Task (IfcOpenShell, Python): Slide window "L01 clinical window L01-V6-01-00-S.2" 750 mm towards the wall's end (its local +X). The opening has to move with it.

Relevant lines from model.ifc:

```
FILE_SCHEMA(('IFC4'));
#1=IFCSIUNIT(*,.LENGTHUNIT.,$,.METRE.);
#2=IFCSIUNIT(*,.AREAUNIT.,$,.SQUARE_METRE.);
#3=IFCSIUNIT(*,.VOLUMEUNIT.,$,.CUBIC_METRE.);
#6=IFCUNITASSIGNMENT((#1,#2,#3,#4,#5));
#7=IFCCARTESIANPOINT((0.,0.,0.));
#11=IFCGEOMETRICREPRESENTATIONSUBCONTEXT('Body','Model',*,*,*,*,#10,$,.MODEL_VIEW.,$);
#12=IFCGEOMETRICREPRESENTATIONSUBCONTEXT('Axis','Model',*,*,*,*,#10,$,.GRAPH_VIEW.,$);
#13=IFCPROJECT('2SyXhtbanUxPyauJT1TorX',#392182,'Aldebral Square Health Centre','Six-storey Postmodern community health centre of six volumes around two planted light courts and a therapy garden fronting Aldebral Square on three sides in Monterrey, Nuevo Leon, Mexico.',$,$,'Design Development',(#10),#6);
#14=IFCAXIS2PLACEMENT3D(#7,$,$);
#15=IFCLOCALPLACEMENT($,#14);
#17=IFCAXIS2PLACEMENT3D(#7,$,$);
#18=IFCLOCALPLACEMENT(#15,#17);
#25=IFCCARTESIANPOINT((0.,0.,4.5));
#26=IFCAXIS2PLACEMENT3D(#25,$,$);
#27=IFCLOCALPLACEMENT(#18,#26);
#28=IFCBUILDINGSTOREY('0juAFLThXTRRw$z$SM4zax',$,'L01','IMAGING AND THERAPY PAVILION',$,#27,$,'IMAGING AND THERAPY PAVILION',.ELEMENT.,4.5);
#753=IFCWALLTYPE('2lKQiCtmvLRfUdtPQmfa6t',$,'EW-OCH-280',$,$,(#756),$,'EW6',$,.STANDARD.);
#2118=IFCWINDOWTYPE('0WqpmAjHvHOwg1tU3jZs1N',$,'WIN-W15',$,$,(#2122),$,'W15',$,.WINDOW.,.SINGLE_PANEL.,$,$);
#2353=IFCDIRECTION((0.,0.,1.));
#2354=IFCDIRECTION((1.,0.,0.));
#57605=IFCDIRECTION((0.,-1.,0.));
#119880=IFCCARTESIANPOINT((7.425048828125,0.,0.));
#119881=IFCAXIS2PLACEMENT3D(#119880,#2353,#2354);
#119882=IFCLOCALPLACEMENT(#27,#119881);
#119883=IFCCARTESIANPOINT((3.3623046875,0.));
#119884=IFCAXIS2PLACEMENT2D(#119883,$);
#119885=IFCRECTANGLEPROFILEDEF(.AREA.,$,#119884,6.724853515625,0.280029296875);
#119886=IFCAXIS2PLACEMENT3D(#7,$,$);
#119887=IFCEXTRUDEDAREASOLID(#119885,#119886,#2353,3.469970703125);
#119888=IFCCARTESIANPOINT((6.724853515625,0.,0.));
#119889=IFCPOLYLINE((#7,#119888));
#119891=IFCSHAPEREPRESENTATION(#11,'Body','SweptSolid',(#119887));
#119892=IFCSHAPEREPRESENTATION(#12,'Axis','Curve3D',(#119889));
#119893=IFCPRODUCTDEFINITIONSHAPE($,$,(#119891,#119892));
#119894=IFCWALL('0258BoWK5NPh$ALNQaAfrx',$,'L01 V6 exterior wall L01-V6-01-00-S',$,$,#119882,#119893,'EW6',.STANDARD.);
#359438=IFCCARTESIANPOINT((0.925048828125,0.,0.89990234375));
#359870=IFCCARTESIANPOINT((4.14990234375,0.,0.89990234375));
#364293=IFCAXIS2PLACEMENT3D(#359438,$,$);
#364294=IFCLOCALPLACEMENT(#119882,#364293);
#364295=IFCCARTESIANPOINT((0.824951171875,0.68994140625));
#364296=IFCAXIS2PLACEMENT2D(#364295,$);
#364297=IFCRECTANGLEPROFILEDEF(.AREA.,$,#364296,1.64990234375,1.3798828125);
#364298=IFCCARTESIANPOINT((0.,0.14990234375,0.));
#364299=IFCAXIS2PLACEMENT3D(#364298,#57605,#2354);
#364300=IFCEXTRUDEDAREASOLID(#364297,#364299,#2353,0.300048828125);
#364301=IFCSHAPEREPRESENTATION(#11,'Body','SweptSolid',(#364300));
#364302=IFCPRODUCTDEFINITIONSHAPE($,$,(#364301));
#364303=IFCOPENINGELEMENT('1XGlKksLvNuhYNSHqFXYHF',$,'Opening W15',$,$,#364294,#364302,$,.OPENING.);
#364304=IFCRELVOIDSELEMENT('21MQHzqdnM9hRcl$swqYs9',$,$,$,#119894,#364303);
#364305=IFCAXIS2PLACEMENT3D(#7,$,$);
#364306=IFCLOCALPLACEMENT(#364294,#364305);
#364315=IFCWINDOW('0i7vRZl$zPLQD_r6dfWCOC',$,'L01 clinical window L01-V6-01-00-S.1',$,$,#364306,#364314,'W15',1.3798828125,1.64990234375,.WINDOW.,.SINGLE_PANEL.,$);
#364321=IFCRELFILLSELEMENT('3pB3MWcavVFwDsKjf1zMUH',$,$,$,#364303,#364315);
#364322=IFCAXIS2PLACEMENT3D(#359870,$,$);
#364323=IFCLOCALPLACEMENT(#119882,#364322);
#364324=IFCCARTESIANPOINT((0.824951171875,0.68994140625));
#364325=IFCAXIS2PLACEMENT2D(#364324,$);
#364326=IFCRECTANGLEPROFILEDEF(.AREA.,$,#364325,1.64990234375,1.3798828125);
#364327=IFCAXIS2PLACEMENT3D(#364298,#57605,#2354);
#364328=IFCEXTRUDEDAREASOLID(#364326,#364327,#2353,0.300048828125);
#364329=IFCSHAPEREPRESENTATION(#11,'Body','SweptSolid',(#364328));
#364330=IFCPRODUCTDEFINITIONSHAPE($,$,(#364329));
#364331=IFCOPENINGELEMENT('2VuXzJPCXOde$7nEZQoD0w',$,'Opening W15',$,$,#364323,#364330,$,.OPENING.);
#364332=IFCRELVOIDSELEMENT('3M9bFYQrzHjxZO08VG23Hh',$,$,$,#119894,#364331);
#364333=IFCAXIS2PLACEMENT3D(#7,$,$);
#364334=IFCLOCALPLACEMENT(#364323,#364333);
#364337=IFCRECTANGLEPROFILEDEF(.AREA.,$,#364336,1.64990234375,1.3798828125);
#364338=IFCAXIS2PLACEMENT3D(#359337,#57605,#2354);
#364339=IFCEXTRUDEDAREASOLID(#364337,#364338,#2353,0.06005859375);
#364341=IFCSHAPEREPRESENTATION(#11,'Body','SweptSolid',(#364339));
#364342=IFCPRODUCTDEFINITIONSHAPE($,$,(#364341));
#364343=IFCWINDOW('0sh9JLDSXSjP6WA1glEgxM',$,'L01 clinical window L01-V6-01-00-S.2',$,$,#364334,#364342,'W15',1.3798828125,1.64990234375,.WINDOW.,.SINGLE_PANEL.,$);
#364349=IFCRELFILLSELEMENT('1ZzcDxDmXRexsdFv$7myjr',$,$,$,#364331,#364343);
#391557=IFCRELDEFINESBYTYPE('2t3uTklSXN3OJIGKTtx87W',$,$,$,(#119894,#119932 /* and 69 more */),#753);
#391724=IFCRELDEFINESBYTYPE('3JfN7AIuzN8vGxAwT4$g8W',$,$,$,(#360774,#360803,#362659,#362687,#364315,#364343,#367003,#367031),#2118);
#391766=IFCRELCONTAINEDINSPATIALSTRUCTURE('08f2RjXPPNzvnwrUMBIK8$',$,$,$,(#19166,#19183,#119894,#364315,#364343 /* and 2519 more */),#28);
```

```python
import ifcopenshell
import ifcopenshell.api.geometry
import ifcopenshell.util.placement
import ifcopenshell.util.unit

model = ifcopenshell.open("model.ifc")
unit_scale = ifcopenshell.util.unit.calculate_unit_scale(model)

window = model.by_guid("0sh9JLDSXSjP6WA1glEgxM")
opening = window.FillsVoids[0].RelatingOpeningElement
wall = opening.VoidsElements[0].RelatingBuildingElement

wall_matrix = ifcopenshell.util.placement.get_local_placement(wall.ObjectPlacement)
shift = wall_matrix[:3, 0] * 0.75 / unit_scale
before = ifcopenshell.util.placement.get_local_placement(window.ObjectPlacement)[:3, 3].copy()

# The window is placed relative to its opening, so it follows when the opening moves.
matrix = ifcopenshell.util.placement.get_local_placement(opening.ObjectPlacement)
matrix[:3, 3] += shift
ifcopenshell.api.geometry.edit_object_placement(
    model, product=opening, matrix=matrix, is_si=False, should_transform_children=True
)

after = ifcopenshell.util.placement.get_local_placement(window.ObjectPlacement)[:3, 3]
print("window moved by", (after - before).round(3) + 0.0)

model.write("model-out.ifc")
```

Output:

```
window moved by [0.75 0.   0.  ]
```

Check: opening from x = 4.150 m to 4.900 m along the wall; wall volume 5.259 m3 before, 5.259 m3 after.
